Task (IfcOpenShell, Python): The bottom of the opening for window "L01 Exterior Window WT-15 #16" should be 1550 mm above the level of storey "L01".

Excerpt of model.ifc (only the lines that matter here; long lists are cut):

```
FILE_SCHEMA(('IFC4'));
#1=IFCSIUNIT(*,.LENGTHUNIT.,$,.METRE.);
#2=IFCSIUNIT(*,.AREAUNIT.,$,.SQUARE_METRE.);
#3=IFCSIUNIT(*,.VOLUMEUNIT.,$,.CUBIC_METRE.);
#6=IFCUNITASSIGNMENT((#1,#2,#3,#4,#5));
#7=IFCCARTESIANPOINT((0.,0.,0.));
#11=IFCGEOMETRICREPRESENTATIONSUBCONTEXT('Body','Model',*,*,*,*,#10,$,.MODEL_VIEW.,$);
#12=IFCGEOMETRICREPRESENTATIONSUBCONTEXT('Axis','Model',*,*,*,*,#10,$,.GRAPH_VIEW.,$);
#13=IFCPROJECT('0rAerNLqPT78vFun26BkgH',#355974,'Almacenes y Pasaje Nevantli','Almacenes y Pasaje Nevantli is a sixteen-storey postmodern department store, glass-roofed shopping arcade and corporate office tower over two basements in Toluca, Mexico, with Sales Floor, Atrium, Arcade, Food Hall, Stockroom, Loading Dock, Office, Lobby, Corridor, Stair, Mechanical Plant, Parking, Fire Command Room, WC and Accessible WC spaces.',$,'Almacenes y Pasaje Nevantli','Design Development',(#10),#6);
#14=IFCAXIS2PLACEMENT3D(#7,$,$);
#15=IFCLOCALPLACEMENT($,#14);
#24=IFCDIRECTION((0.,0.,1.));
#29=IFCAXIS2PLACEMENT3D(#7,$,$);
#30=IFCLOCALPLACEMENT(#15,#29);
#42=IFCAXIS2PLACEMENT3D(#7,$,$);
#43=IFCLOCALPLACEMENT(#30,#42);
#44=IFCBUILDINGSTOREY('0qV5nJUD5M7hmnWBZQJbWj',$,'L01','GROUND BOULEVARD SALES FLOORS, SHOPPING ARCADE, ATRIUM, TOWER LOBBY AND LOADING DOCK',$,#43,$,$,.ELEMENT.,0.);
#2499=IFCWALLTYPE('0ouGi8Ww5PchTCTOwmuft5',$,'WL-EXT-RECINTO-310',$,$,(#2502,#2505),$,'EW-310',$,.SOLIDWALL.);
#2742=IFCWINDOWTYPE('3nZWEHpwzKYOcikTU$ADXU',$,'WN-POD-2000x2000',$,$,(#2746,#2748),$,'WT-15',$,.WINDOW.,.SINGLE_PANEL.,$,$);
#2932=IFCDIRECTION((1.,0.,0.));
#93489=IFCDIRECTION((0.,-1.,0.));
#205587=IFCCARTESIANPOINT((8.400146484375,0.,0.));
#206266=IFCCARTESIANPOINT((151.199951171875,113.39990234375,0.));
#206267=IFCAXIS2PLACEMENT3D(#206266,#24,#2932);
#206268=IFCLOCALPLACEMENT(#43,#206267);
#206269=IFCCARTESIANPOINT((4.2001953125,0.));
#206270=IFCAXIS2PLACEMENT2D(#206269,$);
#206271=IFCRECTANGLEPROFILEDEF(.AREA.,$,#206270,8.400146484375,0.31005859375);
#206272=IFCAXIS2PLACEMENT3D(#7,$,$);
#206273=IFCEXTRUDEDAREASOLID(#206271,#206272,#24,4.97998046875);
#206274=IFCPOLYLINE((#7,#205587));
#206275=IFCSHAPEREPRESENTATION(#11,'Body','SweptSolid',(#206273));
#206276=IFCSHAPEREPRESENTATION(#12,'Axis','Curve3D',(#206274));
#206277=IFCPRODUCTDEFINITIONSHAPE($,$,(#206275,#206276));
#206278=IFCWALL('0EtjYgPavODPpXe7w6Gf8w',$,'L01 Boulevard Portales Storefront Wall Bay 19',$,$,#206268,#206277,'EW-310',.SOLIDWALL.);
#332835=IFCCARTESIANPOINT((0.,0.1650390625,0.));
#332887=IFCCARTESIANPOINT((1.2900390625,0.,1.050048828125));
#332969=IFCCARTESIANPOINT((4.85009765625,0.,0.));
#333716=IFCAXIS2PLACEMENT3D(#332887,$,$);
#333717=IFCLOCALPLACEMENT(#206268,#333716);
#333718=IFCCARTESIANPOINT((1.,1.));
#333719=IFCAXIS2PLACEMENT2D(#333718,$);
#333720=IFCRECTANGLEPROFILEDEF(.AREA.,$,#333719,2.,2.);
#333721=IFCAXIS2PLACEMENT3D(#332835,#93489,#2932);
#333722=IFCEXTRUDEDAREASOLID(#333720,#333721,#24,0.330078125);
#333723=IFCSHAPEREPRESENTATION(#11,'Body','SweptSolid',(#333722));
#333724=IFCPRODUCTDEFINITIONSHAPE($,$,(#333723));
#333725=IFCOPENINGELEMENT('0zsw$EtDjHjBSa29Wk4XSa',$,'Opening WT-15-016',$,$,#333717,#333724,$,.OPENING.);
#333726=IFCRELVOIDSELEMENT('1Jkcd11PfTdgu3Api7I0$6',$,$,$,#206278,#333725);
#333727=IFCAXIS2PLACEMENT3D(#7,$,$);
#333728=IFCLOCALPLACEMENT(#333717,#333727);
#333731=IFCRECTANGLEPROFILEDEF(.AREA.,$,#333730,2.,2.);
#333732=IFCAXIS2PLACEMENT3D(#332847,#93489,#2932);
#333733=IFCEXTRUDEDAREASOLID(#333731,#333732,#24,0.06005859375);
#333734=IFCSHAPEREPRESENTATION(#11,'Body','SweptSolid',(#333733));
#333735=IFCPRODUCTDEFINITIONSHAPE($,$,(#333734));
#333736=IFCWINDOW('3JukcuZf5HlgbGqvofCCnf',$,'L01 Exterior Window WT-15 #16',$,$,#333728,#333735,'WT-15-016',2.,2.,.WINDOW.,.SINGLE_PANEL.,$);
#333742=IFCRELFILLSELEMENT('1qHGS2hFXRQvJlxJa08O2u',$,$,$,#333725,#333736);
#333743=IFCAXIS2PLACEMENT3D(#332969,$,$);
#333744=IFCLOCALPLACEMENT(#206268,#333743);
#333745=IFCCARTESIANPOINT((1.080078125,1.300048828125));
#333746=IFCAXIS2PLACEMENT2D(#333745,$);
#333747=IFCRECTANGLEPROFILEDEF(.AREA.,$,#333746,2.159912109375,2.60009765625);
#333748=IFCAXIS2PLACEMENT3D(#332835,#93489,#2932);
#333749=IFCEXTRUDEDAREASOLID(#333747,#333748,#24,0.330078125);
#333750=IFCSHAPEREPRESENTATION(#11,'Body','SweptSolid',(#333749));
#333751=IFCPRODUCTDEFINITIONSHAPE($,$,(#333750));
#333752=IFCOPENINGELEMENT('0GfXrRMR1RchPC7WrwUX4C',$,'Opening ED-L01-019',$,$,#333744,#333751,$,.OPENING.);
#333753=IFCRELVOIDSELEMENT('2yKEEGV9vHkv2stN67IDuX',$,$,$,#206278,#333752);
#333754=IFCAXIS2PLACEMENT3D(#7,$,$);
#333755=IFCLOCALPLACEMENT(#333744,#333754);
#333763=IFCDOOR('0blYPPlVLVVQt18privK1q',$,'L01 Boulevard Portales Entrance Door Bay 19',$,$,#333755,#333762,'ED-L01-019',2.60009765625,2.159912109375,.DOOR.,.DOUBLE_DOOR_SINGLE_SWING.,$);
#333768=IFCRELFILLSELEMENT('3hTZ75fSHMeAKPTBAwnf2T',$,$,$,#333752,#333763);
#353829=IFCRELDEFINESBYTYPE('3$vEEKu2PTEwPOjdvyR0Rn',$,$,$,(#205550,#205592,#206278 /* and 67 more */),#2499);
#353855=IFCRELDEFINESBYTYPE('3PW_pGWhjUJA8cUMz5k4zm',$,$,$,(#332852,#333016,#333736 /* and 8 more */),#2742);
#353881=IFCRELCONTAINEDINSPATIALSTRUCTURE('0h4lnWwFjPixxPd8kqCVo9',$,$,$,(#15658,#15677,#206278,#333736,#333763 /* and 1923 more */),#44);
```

```python
import numpy as np
import ifcopenshell
import ifcopenshell.api.geometry
import ifcopenshell.geom
import ifcopenshell.util.element
import ifcopenshell.util.placement
import ifcopenshell.util.shape
import ifcopenshell.util.unit

model = ifcopenshell.open("model.ifc")
unit_scale = ifcopenshell.util.unit.calculate_unit_scale(model)

window = model.by_guid("3JukcuZf5HlgbGqvofCCnf")
opening = window.FillsVoids[0].RelatingOpeningElement
storey = ifcopenshell.util.element.get_container(window, ifc_class="IfcBuildingStorey")
level = ifcopenshell.util.placement.get_local_placement(storey.ObjectPlacement)[2, 3]

# The opening's origin need not be at the sill, so measure its lowest point.
shape = ifcopenshell.geom.create_shape(ifcopenshell.geom.settings(), opening)
bottom = ifcopenshell.util.shape.get_shape_bottom_elevation(shape, shape.geometry) / unit_scale
dz = level + 1.55 / unit_scale - bottom

shift = np.array([0.0, 0.0, dz])
# The window is placed relative to its opening, so it follows when the opening moves.
matrix = ifcopenshell.util.placement.get_local_placement(opening.ObjectPlacement)
matrix[:3, 3] += shift
ifcopenshell.api.geometry.edit_object_placement(
    model, product=opening, matrix=matrix, is_si=False, should_transform_children=True
)

print(f"moved by {dz * unit_scale:+.3f} m")

model.write("model_edited.ifc")
```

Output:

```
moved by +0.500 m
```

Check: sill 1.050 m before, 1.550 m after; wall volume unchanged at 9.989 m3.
